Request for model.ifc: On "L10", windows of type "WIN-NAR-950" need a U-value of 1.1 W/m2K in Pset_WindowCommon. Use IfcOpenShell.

First a look at what the model holds.

```python
import ifcopenshell
import ifcopenshell.util.element

model = ifcopenshell.open("model.ifc")
print(model.schema)
storey = next(s for s in model.by_type("IfcBuildingStorey") if s.Name == "L10")
windows = [e for e in ifcopenshell.util.element.get_decomposition(storey) if e.is_a("IfcWindow")]
seen = {}
for e in windows:
    element_type = ifcopenshell.util.element.get_type(e)
    key = (element_type.Name if element_type != e and element_type else None, ifcopenshell.util.element.get_pset(e, "Pset_WindowCommon", "ThermalTransmittance"))
    seen[key] = seen.get(key, 0) + 1
for (name, value), count in sorted(seen.items(), key=str):
    print(count, "x", name, "|", value)
```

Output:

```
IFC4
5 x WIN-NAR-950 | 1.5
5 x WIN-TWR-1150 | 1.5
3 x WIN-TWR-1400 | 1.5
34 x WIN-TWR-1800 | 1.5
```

```python
import ifcopenshell
import ifcopenshell.api.pset
import ifcopenshell.util.element

model = ifcopenshell.open("model.ifc")

storey = next(s for s in model.by_type("IfcBuildingStorey") if s.Name == "L10")
windows = [e for e in ifcopenshell.util.element.get_decomposition(storey) if e.is_a("IfcWindow")]

count = 0
for e in windows:
    element_type = ifcopenshell.util.element.get_type(e)
    if element_type in (None, e) or element_type.Name != "WIN-NAR-950":
        continue
    found = ifcopenshell.util.element.get_pset(e, "Pset_WindowCommon", should_inherit=False)
    if found:
        pset = model.by_id(found["id"])
        if len(ifcopenshell.util.element.get_elements_by_pset(pset)) > 1:
            pset = ifcopenshell.api.pset.unshare_pset(model, products=[e], pset=pset)[0]
    else:
        pset = ifcopenshell.api.pset.add_pset(model, product=e, name="Pset_WindowCommon")
    ifcopenshell.api.pset.edit_pset(model, pset=pset, properties={"ThermalTransmittance": 1.1})
    count += 1

print(count, "windows updated")

model.write("model_edited.ifc")
```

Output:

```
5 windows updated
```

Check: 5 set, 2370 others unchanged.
